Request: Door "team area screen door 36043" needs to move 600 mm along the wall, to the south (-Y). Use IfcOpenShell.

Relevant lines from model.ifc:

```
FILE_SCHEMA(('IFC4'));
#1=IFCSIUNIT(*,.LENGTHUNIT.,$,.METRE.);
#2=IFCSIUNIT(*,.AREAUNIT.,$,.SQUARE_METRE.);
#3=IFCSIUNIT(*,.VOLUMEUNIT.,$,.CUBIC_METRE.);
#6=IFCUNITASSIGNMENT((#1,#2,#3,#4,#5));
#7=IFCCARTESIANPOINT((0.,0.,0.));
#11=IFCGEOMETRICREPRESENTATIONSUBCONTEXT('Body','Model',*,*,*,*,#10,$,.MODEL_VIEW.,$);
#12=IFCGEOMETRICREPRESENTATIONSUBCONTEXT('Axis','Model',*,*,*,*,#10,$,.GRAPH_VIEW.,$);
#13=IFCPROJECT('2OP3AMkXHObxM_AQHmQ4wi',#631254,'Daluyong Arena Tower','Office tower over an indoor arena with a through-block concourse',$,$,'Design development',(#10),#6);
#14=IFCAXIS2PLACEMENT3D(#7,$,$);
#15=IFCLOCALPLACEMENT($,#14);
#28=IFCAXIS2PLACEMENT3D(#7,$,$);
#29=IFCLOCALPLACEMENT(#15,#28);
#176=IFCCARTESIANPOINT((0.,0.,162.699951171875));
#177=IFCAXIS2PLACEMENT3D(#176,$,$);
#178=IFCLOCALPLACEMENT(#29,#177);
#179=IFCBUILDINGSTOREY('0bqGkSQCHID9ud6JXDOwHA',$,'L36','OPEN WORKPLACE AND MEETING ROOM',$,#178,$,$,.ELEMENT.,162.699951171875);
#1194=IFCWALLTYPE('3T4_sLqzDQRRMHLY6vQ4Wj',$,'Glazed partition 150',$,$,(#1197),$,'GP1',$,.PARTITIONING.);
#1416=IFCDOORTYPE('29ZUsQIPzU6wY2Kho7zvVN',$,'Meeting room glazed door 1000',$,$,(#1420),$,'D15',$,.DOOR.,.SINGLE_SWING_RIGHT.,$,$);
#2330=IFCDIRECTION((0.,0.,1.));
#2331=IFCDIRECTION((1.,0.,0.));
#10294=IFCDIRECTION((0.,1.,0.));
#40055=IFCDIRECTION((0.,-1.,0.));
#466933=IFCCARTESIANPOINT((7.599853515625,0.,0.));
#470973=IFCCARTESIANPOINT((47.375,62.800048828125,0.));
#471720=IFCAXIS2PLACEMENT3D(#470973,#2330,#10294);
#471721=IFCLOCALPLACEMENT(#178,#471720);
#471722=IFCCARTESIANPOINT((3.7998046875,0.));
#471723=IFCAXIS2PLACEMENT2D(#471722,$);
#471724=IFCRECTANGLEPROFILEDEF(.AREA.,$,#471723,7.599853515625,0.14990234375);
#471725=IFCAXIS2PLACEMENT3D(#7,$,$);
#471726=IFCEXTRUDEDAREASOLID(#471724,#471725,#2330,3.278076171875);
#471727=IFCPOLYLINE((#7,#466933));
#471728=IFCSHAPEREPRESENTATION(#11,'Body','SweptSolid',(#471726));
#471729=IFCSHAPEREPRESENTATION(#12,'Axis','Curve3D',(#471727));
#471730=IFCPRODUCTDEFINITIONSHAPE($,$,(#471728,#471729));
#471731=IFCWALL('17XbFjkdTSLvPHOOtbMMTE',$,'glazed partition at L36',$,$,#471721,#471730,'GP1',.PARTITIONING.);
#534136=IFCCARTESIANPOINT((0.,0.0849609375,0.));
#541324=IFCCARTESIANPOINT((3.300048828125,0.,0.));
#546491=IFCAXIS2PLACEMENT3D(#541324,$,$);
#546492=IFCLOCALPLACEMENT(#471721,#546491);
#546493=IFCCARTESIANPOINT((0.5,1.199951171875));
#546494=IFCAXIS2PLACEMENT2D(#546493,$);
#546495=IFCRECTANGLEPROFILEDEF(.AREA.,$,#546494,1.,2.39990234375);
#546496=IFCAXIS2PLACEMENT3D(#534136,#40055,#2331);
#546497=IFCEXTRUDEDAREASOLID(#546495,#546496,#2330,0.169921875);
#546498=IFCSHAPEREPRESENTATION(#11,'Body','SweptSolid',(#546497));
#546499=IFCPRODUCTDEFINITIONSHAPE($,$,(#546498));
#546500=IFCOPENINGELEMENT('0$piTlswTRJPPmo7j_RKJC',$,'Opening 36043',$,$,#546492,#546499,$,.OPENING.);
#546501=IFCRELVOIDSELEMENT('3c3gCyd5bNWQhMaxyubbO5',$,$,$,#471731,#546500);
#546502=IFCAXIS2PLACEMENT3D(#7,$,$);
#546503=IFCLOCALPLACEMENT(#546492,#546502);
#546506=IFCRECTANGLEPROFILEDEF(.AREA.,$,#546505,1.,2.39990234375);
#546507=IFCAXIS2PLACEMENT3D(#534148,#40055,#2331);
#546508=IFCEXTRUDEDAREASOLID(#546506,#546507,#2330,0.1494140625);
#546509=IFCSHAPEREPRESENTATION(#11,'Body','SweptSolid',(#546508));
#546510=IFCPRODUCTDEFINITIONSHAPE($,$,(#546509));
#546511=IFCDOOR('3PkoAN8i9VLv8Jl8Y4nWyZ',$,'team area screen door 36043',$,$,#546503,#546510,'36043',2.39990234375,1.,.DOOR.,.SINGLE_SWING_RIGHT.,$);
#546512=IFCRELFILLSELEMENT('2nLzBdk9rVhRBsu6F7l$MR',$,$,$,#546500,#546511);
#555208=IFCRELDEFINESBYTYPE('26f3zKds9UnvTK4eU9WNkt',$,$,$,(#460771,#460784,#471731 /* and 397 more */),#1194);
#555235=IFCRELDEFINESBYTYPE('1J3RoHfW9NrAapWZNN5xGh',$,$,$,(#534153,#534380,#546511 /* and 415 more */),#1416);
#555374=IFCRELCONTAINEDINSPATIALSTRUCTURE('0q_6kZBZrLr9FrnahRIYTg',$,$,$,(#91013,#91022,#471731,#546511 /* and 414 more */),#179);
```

```python
import ifcopenshell
import ifcopenshell.api.geometry
import ifcopenshell.util.placement
import ifcopenshell.util.unit

model = ifcopenshell.open("model.ifc")
unit_scale = ifcopenshell.util.unit.calculate_unit_scale(model)

door = model.by_guid("3PkoAN8i9VLv8Jl8Y4nWyZ")
opening = door.FillsVoids[0].RelatingOpeningElement
wall = opening.VoidsElements[0].RelatingBuildingElement

wall_matrix = ifcopenshell.util.placement.get_local_placement(wall.ObjectPlacement)
shift = wall_matrix[:3, 0] * -0.6 / unit_scale
before = ifcopenshell.util.placement.get_local_placement(door.ObjectPlacement)[:3, 3].copy()

# The door is placed relative to its opening, so it follows when the opening moves.
matrix = ifcopenshell.util.placement.get_local_placement(opening.ObjectPlacement)
matrix[:3, 3] += shift
ifcopenshell.api.geometry.edit_object_placement(
    model, product=opening, matrix=matrix, is_si=False, should_transform_children=True
)

after = ifcopenshell.util.placement.get_local_placement(door.ObjectPlacement)[:3, 3]
print("door moved by", (after - before).round(3) + 0.0)

model.write("model_updated.ifc")
```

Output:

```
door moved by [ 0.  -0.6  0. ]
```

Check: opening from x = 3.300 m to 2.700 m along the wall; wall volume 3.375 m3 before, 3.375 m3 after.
